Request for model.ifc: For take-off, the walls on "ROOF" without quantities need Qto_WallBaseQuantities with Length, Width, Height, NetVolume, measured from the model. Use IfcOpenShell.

First a look at what the model holds.

```python
import ifcopenshell
import ifcopenshell.util.element
import ifcopenshell.util.unit

model = ifcopenshell.open("model.ifc")
print(model.schema)
for unit_type in ("LENGTHUNIT", "AREAUNIT", "VOLUMEUNIT"):
    print(unit_type, ifcopenshell.util.unit.calculate_unit_scale(model, unit_type))
storey = next(s for s in model.by_type("IfcBuildingStorey") if s.Name == "ROOF")
walls = [e for e in ifcopenshell.util.element.get_decomposition(storey) if e.is_a("IfcWall")]
for e in sorted(walls, key=lambda e: e.id()):
    print(e.id(), e.is_a(), e.Name, list(ifcopenshell.util.element.get_psets(e, qtos_only=True)), sep=" | ")
```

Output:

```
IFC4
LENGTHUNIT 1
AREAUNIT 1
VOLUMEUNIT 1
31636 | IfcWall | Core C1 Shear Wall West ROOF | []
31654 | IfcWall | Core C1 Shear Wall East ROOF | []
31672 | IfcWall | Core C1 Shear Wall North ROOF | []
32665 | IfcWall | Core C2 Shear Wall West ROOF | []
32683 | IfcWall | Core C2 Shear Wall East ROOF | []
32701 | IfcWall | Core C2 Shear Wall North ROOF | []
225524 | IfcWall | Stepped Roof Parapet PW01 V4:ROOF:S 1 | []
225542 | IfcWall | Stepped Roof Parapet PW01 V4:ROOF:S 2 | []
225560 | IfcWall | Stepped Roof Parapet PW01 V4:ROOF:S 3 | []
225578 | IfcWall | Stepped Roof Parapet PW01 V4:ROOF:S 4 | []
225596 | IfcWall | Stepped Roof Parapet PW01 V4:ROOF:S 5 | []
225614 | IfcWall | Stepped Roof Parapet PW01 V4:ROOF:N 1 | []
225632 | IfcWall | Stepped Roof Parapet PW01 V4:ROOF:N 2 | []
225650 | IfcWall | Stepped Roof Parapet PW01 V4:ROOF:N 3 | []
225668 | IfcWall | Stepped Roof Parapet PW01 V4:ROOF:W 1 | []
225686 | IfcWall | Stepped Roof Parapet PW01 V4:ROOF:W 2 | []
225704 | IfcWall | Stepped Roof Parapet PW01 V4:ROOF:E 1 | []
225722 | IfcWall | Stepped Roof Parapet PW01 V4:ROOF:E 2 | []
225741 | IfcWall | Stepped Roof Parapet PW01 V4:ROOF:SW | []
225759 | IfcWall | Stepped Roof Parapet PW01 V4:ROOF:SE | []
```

```python
import ifcopenshell
import ifcopenshell.api.pset
import ifcopenshell.geom
import ifcopenshell.util.element
import ifcopenshell.util.shape
import ifcopenshell.util.unit

model = ifcopenshell.open("model.ifc")
unit_scale = ifcopenshell.util.unit.calculate_unit_scale(model)
volume_scale = ifcopenshell.util.unit.calculate_unit_scale(model, "VOLUMEUNIT")
settings = ifcopenshell.geom.settings()

storey = next(s for s in model.by_type("IfcBuildingStorey") if s.Name == "ROOF")
walls = [e for e in ifcopenshell.util.element.get_decomposition(storey) if e.is_a("IfcWall")]

for e in sorted(walls, key=lambda e: e.id()):
    if ifcopenshell.util.element.get_psets(e, qtos_only=True, should_inherit=False):
        continue
    # Geometry comes back in metres, in the element's own axes.
    shape = ifcopenshell.geom.create_shape(settings, e)
    values = {
        "Length": ifcopenshell.util.shape.get_x(shape.geometry) / unit_scale,
        "Width": ifcopenshell.util.shape.get_y(shape.geometry) / unit_scale,
        "Height": ifcopenshell.util.shape.get_z(shape.geometry) / unit_scale,
        "NetVolume": ifcopenshell.util.shape.get_volume(shape.geometry) / volume_scale,
    }
    qto = ifcopenshell.api.pset.add_qto(model, product=e, name="Qto_WallBaseQuantities")
    ifcopenshell.api.pset.edit_qto(model, qto=qto, properties=values)
    print(e.id(), {k: round(v, 3) for k, v in values.items()})

model.write("model_edited.ifc")
```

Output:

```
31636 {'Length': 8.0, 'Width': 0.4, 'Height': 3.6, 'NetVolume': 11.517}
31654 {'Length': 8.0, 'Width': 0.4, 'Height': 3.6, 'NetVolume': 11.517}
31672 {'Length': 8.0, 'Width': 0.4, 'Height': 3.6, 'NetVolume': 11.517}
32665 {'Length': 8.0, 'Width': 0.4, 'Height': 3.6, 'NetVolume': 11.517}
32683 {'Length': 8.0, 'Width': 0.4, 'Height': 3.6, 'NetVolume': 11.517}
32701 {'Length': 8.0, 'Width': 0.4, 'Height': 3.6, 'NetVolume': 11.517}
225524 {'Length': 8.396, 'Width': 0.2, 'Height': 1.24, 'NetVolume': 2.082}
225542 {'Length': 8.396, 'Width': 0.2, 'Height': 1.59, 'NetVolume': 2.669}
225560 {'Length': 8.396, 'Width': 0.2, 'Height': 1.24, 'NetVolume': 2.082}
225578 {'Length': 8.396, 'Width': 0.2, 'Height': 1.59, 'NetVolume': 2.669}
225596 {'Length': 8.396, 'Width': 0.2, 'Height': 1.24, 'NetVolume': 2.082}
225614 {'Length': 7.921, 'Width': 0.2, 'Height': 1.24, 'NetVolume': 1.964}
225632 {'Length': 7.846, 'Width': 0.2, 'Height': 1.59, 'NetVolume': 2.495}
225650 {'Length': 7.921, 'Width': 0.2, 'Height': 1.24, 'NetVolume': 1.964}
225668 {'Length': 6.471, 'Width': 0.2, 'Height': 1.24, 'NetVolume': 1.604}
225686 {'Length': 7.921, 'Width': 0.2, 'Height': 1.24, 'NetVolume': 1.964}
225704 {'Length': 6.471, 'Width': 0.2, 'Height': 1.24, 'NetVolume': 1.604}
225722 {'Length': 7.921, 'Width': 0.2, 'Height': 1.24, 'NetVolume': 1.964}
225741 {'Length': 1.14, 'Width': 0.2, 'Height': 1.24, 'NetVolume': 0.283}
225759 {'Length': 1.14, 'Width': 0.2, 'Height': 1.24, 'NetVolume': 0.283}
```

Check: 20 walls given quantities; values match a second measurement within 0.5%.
